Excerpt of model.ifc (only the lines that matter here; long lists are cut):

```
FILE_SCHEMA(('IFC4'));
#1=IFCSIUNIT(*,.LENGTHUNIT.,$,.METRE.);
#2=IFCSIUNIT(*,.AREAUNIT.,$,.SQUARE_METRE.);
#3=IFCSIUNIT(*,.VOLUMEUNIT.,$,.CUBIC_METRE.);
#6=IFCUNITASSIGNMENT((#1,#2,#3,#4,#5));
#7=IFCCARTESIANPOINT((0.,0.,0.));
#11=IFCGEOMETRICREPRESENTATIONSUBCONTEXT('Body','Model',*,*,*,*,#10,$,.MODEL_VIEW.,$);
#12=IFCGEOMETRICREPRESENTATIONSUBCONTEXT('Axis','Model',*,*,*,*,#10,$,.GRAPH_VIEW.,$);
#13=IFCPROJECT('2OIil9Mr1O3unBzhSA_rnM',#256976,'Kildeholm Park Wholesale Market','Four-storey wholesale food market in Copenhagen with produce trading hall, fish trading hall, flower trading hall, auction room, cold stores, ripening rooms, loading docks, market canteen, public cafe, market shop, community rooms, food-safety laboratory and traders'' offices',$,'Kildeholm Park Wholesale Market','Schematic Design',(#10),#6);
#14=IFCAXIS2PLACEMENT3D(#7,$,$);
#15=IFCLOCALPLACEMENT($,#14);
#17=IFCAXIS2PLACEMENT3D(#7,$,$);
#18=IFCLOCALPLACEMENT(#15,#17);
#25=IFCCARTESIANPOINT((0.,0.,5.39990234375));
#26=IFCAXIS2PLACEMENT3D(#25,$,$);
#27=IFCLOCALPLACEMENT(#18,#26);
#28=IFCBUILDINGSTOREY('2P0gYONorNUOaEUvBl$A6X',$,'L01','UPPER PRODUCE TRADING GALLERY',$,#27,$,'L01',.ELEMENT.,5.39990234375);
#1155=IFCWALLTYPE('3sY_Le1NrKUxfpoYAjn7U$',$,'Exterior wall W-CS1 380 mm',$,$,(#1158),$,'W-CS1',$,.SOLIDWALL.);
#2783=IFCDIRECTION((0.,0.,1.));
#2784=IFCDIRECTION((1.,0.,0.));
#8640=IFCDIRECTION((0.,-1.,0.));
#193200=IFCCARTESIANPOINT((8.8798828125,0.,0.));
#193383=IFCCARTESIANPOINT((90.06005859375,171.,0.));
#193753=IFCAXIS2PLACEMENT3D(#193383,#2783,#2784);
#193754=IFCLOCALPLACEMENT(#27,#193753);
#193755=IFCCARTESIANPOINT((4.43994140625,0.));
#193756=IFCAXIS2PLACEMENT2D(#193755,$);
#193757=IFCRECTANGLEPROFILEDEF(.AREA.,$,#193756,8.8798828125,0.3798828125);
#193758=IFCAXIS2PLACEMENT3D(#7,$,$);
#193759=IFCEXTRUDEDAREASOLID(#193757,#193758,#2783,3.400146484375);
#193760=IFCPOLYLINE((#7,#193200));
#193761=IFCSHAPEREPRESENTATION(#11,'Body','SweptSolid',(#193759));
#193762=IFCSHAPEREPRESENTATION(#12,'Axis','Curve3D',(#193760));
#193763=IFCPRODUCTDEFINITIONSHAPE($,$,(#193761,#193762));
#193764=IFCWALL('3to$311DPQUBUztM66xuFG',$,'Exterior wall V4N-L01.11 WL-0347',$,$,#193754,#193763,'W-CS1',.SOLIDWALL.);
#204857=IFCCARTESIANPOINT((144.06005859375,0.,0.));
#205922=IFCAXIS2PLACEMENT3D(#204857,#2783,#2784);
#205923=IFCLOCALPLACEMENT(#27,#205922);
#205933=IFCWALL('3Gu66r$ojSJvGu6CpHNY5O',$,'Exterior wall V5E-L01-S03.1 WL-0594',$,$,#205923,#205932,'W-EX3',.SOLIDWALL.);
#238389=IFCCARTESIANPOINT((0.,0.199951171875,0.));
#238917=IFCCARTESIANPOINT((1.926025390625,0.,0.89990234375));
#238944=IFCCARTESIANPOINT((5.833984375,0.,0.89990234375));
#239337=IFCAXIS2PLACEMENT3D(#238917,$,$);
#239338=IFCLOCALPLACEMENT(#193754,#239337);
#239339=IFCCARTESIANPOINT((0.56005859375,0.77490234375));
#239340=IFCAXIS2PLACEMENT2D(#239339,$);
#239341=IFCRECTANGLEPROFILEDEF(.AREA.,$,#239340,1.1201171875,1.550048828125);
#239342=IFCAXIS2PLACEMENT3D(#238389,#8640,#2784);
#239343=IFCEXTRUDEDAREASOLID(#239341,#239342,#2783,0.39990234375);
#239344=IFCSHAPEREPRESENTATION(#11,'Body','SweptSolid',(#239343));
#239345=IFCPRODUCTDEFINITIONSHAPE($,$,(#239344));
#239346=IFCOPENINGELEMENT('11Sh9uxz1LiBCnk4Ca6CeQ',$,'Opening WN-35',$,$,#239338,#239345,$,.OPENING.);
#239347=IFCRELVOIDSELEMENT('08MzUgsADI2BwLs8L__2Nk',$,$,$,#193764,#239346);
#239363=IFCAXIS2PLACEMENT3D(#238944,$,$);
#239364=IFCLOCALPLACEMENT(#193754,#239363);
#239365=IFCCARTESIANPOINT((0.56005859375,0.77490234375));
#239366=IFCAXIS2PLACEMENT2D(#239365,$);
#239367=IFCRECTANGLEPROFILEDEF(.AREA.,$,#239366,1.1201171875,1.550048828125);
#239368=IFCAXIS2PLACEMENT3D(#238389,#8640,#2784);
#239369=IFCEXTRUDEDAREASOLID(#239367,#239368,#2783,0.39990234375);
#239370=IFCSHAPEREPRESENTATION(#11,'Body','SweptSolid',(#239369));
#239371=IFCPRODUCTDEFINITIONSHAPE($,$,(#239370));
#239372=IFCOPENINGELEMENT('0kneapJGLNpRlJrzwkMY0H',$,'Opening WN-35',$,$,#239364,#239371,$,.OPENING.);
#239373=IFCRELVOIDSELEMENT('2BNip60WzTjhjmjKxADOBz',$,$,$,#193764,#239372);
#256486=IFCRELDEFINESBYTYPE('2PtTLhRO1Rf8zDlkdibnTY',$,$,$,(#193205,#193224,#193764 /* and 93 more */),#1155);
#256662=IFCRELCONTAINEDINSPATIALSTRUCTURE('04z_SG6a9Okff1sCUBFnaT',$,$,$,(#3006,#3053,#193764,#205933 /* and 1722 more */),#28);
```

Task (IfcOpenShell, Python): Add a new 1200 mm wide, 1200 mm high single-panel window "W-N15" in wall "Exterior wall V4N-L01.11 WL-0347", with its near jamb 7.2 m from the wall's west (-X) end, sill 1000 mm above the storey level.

```python
import numpy as np
import ifcopenshell
import ifcopenshell.api.feature
import ifcopenshell.api.geometry
import ifcopenshell.api.root
import ifcopenshell.api.spatial
import ifcopenshell.geom
import ifcopenshell.util.element
import ifcopenshell.util.placement
import ifcopenshell.util.representation
import ifcopenshell.util.shape
import ifcopenshell.util.unit

model = ifcopenshell.open("model.ifc")
unit_scale = ifcopenshell.util.unit.calculate_unit_scale(model)
settings = ifcopenshell.geom.settings()


def volume(element):
    """Net volume in cubic metres, openings subtracted."""
    shape = ifcopenshell.geom.create_shape(settings, element)
    return ifcopenshell.util.shape.get_volume(shape.geometry)


wall = model.by_guid("3to$311DPQUBUztM66xuFG")
storey = ifcopenshell.util.element.get_container(wall, ifc_class="IfcBuildingStorey")
context = ifcopenshell.util.representation.get_context(model, "Model", "Body", "MODEL_VIEW")
before = volume(wall)

width, height, from_end, sill = 1.2, 1.2, 7.2, 1  # metres

# The wall runs along its own X axis, and the end named is its -X end.
wall_shape = ifcopenshell.geom.create_shape(settings, wall)
x, y, z = ifcopenshell.util.shape.get_vertices(wall_shape.geometry).T
start = x.min() + from_end
face, thickness = float(y.min()), float(y.max() - y.min())
wall_matrix = ifcopenshell.util.placement.get_local_placement(wall.ObjectPlacement)
level = ifcopenshell.util.placement.get_local_placement(storey.ObjectPlacement)[2, 3]


def in_wall(x, y):
    """Placement at x, y metres in the wall's axes, at sill height."""
    matrix = wall_matrix.copy()
    matrix[:, 3] = wall_matrix @ np.array([x / unit_scale, y / unit_scale, 0.0, 1.0])
    matrix[2, 3] = level + sill / unit_scale
    return matrix


# Opening: a box that overshoots both wall faces by 50 mm.
opening = ifcopenshell.api.root.create_entity(model, ifc_class="IfcOpeningElement", predefined_type="OPENING")
box = ifcopenshell.api.geometry.add_wall_representation(
    model, context=context, length=width, height=height, thickness=thickness + 0.1
)
ifcopenshell.api.geometry.assign_representation(model, product=opening, representation=box)
ifcopenshell.api.geometry.edit_object_placement(model, product=opening, matrix=in_wall(start, face - 0.05), is_si=False)
ifcopenshell.api.feature.add_feature(model, feature=opening, element=wall)

window = ifcopenshell.api.root.create_entity(model, ifc_class="IfcWindow", name="W-N15", predefined_type="WINDOW")
window.OverallWidth, window.OverallHeight = width / unit_scale, height / unit_scale
window.PartitioningType = "SINGLE_PANEL"
body = ifcopenshell.api.geometry.add_window_representation(
    model,
    context=context,
    overall_width=window.OverallWidth,
    overall_height=window.OverallHeight,
    partition_type="SINGLE_PANEL",
)
ifcopenshell.api.geometry.assign_representation(model, product=window, representation=body)
ifcopenshell.api.spatial.assign_container(model, products=[window], relating_structure=storey)
ifcopenshell.api.feature.add_filling(model, opening=opening, element=window)

# Centre the window in the wall's thickness.
ifcopenshell.api.geometry.edit_object_placement(model, product=window, matrix=in_wall(start, face), is_si=False)
window_shape = ifcopenshell.geom.create_shape(settings, window)
depth = ifcopenshell.util.shape.get_vertices(window_shape.geometry)[:, 1]
offset = face + thickness / 2 - (depth.min() + depth.max()) / 2
ifcopenshell.api.geometry.edit_object_placement(model, product=window, matrix=in_wall(start, offset), is_si=False)

after = volume(wall)

print(f"wall volume {before:.3f} -> {after:.3f} m3")

model.write("model_updated.ifc")
```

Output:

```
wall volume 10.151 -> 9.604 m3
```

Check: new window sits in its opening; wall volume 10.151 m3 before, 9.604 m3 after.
